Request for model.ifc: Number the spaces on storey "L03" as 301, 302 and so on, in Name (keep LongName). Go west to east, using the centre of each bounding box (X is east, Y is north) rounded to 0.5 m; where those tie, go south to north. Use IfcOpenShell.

First a look at what the model holds.

```python
import ifcopenshell
import ifcopenshell.util.element
import ifcopenshell.util.placement

model = ifcopenshell.open("model.ifc")
print(model.schema)
storey = next(s for s in model.by_type("IfcBuildingStorey") if s.Name == "L03")
spaces = [e for e in ifcopenshell.util.element.get_decomposition(storey) if e.is_a("IfcSpace")]
for e in sorted(spaces, key=lambda e: e.id()):
    origin = ifcopenshell.util.placement.get_local_placement(e.ObjectPlacement)[:3, 3]
    print(e.id(), e.Name, e.LongName, origin.round(2) + 0.0, sep=" | ")
```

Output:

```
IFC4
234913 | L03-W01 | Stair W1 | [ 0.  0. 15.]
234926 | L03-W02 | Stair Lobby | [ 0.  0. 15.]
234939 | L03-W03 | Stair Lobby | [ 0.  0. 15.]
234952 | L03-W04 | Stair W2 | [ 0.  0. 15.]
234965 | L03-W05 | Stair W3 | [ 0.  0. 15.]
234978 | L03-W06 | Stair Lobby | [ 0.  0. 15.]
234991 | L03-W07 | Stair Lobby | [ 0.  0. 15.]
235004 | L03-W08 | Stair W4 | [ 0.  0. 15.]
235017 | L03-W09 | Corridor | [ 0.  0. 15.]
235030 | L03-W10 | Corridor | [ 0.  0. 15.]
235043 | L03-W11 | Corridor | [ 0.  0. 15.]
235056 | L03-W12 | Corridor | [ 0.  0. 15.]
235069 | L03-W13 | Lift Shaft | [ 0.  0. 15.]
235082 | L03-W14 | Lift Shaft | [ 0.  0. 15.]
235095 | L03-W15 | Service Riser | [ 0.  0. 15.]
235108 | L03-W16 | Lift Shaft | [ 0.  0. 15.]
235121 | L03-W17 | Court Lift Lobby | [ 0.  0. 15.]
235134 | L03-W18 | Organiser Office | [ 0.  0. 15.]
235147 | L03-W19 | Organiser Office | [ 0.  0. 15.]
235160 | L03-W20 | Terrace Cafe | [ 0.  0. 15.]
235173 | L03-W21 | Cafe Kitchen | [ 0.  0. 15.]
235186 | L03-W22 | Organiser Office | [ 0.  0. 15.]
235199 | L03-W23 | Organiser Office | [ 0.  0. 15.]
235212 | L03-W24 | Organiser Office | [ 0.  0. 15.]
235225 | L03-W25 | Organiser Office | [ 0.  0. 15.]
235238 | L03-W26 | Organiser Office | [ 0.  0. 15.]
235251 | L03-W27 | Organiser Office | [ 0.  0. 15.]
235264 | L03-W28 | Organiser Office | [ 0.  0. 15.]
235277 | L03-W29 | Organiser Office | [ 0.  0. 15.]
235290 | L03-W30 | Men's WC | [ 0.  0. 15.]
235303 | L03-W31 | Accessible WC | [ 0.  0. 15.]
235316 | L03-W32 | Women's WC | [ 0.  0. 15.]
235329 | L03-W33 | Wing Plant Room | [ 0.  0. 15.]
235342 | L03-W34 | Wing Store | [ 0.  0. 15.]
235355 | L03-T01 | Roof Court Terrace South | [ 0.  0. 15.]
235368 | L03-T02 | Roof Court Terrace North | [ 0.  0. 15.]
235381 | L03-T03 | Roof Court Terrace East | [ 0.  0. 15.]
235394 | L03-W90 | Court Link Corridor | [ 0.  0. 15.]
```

```python
import ifcopenshell
import ifcopenshell.geom
import ifcopenshell.util.element
import ifcopenshell.util.shape

model = ifcopenshell.open("model.ifc")
settings = ifcopenshell.geom.settings()
settings.set("use-world-coords", True)


def centre(element):
    shape = ifcopenshell.geom.create_shape(settings, element)
    return ifcopenshell.util.shape.get_bbox_centroid(shape.geometry)


storey = next(s for s in model.by_type("IfcBuildingStorey") if s.Name == "L03")
spaces = [e for e in ifcopenshell.util.element.get_decomposition(storey) if e.is_a("IfcSpace")]

# Insertion points can sit at a corner or the storey origin, so sort by the geometry (in metres).
centres = {e: centre(e) for e in spaces}
spaces.sort(key=lambda e: (round(centres[e][0] / 0.5), centres[e][1]))

for i, e in enumerate(spaces, start=1):
    number = f"3{i:02d}"
    e.Name = number
    print(e.id(), number)

model.write("model_rev.ifc")
```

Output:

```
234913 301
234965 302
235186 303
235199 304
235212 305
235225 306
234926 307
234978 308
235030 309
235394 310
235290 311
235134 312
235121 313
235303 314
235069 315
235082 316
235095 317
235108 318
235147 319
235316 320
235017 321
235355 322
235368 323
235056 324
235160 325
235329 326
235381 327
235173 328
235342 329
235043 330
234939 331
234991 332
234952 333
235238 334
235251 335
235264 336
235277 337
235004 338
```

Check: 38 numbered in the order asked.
